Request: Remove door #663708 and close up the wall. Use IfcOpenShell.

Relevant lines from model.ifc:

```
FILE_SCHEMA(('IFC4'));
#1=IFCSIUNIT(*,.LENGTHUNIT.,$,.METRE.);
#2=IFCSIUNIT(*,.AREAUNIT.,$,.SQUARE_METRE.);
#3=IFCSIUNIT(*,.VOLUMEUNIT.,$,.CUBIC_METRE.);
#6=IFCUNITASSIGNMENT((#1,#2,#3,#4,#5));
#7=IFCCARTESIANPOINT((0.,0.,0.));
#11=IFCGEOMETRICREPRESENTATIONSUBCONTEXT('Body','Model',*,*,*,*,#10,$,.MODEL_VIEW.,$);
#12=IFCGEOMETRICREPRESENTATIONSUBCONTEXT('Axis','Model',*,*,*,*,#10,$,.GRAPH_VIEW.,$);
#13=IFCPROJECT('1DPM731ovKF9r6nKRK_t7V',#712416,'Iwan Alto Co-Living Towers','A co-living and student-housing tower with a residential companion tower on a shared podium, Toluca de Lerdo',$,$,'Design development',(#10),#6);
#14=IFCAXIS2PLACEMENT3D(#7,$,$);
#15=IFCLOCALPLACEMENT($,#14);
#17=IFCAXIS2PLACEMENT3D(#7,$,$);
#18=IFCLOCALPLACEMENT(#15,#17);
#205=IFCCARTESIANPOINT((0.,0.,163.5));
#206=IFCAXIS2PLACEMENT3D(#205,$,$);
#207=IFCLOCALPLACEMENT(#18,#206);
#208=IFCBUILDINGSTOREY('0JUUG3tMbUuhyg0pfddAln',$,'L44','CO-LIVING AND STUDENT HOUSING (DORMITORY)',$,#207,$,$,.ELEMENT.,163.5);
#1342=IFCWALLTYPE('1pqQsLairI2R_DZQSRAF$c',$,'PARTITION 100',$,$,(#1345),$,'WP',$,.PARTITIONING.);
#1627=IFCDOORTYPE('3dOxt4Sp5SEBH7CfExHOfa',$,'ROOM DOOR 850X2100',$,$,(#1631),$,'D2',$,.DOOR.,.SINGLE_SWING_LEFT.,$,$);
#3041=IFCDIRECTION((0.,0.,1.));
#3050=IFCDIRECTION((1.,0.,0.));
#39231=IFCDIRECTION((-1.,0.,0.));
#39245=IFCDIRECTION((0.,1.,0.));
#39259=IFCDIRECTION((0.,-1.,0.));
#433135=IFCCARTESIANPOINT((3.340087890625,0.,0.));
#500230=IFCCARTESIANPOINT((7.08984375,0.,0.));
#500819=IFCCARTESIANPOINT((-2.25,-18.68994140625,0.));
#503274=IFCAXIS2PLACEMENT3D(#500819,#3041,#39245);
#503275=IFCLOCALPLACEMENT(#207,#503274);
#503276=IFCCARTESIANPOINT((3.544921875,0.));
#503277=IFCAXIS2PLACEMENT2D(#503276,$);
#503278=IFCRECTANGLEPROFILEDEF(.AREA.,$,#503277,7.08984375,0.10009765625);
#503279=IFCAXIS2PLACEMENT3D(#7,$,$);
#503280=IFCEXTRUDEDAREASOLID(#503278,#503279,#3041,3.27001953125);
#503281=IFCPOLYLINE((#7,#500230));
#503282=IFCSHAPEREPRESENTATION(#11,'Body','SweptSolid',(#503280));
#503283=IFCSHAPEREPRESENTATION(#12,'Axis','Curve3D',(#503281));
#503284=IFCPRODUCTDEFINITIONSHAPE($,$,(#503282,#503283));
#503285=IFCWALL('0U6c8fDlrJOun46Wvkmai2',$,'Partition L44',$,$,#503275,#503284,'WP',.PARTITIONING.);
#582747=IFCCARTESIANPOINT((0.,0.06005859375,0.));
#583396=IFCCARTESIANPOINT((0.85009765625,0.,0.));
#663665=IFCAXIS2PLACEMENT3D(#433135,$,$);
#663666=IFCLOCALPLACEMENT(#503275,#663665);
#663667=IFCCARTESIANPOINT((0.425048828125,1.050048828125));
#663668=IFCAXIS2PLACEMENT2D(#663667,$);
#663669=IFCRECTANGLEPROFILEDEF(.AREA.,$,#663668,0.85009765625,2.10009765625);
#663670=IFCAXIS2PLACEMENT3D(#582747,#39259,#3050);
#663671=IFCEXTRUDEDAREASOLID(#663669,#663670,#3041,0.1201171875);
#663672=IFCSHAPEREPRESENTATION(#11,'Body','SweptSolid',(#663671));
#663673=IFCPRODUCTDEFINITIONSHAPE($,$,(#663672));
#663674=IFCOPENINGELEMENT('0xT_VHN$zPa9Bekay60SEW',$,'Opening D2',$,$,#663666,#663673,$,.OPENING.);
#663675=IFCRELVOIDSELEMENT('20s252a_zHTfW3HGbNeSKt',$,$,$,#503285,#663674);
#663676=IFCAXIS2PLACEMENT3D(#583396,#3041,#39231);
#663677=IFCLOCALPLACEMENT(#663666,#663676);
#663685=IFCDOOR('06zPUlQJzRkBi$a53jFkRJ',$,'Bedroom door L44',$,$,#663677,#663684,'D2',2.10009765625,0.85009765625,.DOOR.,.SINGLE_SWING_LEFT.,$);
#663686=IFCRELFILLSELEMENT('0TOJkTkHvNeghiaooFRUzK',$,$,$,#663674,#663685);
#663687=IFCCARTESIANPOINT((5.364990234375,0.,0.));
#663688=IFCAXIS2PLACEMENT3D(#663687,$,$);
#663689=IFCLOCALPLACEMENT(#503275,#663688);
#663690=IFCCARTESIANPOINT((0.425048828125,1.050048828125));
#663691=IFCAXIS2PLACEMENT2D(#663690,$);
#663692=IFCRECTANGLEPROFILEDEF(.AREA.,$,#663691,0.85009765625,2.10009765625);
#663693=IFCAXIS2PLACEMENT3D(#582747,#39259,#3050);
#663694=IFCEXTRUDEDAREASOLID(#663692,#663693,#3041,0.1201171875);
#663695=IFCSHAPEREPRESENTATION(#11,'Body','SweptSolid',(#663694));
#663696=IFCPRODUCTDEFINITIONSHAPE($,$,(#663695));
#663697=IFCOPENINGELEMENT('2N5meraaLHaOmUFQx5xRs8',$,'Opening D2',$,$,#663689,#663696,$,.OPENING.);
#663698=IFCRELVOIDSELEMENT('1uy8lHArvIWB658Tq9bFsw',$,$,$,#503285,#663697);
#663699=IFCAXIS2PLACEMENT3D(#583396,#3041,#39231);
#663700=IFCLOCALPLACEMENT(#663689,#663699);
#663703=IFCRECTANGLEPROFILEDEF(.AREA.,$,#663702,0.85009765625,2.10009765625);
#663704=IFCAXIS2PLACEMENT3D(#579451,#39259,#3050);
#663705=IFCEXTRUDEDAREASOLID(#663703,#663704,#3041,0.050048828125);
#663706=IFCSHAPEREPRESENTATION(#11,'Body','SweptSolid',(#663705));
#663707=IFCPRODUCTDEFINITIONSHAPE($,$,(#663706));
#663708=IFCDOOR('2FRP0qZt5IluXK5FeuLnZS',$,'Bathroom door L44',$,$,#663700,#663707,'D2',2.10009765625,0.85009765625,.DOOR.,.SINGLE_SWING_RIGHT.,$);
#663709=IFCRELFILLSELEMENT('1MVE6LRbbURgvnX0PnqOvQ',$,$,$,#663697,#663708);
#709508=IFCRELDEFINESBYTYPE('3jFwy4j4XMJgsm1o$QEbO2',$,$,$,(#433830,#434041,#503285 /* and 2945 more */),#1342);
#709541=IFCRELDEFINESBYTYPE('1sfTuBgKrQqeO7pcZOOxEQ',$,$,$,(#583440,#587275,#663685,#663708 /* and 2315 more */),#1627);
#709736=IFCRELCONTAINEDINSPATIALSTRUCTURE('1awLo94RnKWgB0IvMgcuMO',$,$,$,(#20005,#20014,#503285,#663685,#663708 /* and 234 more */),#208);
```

```python
import ifcopenshell
import ifcopenshell.api.feature
import ifcopenshell.api.root
import ifcopenshell.geom
import ifcopenshell.util.shape

model = ifcopenshell.open("model.ifc")
settings = ifcopenshell.geom.settings()


def volume(element):
    """Net volume in cubic metres, openings subtracted."""
    shape = ifcopenshell.geom.create_shape(settings, element)
    return ifcopenshell.util.shape.get_volume(shape.geometry)


door = model.by_guid("2FRP0qZt5IluXK5FeuLnZS")
opening = door.FillsVoids[0].RelatingOpeningElement
wall = opening.VoidsElements[0].RelatingBuildingElement
before = volume(wall)

ifcopenshell.api.root.remove_product(model, product=door)
ifcopenshell.api.feature.remove_feature(model, feature=opening)

after = volume(wall)

print(f"wall volume {before:.3f} -> {after:.3f} m3")

model.write("model_rev.ifc")
```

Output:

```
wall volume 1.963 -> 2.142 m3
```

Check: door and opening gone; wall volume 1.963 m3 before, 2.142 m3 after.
